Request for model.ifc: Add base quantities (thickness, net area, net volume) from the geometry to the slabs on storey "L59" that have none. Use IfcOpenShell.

First a look at what the model holds.

```python
import ifcopenshell
import ifcopenshell.util.element
import ifcopenshell.util.unit

model = ifcopenshell.open("model.ifc")
print(model.schema)
for unit_type in ("LENGTHUNIT", "AREAUNIT", "VOLUMEUNIT"):
    print(unit_type, ifcopenshell.util.unit.calculate_unit_scale(model, unit_type))
storey = next(s for s in model.by_type("IfcBuildingStorey") if s.Name == "L59")
slabs = [e for e in ifcopenshell.util.element.get_decomposition(storey) if e.is_a("IfcSlab")]
for e in sorted(slabs, key=lambda e: e.id()):
    print(e.id(), e.is_a(), e.Name, list(ifcopenshell.util.element.get_psets(e, qtos_only=True)), sep=" | ")
```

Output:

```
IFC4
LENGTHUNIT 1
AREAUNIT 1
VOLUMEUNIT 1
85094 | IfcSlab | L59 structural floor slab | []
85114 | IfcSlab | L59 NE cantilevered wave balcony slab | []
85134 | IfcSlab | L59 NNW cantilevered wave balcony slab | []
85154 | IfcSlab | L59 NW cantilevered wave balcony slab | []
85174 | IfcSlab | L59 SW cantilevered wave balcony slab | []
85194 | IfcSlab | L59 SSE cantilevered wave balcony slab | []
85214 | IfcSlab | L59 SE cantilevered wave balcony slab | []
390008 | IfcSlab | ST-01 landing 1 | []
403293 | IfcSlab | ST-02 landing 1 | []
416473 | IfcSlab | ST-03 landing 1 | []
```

```python
import ifcopenshell
import ifcopenshell.api.pset
import ifcopenshell.geom
import ifcopenshell.util.element
import ifcopenshell.util.shape
import ifcopenshell.util.unit

model = ifcopenshell.open("model.ifc")
unit_scale = ifcopenshell.util.unit.calculate_unit_scale(model)
area_scale = ifcopenshell.util.unit.calculate_unit_scale(model, "AREAUNIT")
volume_scale = ifcopenshell.util.unit.calculate_unit_scale(model, "VOLUMEUNIT")
settings = ifcopenshell.geom.settings()

storey = next(s for s in model.by_type("IfcBuildingStorey") if s.Name == "L59")
slabs = [e for e in ifcopenshell.util.element.get_decomposition(storey) if e.is_a("IfcSlab")]

for e in sorted(slabs, key=lambda e: e.id()):
    if ifcopenshell.util.element.get_psets(e, qtos_only=True, should_inherit=False):
        continue
    # Geometry comes back in metres, in the element's own axes.
    shape = ifcopenshell.geom.create_shape(settings, e)
    values = {
        "Width": ifcopenshell.util.shape.get_z(shape.geometry) / unit_scale,
        "NetArea": ifcopenshell.util.shape.get_footprint_area(shape.geometry) / area_scale,
        "NetVolume": ifcopenshell.util.shape.get_volume(shape.geometry) / volume_scale,
    }
    qto = ifcopenshell.api.pset.add_qto(model, product=e, name="Qto_SlabBaseQuantities")
    ifcopenshell.api.pset.edit_qto(model, qto=qto, properties=values)
    print(e.id(), {k: round(v, 3) for k, v in values.items()})

model.write("model_rev.ifc")
```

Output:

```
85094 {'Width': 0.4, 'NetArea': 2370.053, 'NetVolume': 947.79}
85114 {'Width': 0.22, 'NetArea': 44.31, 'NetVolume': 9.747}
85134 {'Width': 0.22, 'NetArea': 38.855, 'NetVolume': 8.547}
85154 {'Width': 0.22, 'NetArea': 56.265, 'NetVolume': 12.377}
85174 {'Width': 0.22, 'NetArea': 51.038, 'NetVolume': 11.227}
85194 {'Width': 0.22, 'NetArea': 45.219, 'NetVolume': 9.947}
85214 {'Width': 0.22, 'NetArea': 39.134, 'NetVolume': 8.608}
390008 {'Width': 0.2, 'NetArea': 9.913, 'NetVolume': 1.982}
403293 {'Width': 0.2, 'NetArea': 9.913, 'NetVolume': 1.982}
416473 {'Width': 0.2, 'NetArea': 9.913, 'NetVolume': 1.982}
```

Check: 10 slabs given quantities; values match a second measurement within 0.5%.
